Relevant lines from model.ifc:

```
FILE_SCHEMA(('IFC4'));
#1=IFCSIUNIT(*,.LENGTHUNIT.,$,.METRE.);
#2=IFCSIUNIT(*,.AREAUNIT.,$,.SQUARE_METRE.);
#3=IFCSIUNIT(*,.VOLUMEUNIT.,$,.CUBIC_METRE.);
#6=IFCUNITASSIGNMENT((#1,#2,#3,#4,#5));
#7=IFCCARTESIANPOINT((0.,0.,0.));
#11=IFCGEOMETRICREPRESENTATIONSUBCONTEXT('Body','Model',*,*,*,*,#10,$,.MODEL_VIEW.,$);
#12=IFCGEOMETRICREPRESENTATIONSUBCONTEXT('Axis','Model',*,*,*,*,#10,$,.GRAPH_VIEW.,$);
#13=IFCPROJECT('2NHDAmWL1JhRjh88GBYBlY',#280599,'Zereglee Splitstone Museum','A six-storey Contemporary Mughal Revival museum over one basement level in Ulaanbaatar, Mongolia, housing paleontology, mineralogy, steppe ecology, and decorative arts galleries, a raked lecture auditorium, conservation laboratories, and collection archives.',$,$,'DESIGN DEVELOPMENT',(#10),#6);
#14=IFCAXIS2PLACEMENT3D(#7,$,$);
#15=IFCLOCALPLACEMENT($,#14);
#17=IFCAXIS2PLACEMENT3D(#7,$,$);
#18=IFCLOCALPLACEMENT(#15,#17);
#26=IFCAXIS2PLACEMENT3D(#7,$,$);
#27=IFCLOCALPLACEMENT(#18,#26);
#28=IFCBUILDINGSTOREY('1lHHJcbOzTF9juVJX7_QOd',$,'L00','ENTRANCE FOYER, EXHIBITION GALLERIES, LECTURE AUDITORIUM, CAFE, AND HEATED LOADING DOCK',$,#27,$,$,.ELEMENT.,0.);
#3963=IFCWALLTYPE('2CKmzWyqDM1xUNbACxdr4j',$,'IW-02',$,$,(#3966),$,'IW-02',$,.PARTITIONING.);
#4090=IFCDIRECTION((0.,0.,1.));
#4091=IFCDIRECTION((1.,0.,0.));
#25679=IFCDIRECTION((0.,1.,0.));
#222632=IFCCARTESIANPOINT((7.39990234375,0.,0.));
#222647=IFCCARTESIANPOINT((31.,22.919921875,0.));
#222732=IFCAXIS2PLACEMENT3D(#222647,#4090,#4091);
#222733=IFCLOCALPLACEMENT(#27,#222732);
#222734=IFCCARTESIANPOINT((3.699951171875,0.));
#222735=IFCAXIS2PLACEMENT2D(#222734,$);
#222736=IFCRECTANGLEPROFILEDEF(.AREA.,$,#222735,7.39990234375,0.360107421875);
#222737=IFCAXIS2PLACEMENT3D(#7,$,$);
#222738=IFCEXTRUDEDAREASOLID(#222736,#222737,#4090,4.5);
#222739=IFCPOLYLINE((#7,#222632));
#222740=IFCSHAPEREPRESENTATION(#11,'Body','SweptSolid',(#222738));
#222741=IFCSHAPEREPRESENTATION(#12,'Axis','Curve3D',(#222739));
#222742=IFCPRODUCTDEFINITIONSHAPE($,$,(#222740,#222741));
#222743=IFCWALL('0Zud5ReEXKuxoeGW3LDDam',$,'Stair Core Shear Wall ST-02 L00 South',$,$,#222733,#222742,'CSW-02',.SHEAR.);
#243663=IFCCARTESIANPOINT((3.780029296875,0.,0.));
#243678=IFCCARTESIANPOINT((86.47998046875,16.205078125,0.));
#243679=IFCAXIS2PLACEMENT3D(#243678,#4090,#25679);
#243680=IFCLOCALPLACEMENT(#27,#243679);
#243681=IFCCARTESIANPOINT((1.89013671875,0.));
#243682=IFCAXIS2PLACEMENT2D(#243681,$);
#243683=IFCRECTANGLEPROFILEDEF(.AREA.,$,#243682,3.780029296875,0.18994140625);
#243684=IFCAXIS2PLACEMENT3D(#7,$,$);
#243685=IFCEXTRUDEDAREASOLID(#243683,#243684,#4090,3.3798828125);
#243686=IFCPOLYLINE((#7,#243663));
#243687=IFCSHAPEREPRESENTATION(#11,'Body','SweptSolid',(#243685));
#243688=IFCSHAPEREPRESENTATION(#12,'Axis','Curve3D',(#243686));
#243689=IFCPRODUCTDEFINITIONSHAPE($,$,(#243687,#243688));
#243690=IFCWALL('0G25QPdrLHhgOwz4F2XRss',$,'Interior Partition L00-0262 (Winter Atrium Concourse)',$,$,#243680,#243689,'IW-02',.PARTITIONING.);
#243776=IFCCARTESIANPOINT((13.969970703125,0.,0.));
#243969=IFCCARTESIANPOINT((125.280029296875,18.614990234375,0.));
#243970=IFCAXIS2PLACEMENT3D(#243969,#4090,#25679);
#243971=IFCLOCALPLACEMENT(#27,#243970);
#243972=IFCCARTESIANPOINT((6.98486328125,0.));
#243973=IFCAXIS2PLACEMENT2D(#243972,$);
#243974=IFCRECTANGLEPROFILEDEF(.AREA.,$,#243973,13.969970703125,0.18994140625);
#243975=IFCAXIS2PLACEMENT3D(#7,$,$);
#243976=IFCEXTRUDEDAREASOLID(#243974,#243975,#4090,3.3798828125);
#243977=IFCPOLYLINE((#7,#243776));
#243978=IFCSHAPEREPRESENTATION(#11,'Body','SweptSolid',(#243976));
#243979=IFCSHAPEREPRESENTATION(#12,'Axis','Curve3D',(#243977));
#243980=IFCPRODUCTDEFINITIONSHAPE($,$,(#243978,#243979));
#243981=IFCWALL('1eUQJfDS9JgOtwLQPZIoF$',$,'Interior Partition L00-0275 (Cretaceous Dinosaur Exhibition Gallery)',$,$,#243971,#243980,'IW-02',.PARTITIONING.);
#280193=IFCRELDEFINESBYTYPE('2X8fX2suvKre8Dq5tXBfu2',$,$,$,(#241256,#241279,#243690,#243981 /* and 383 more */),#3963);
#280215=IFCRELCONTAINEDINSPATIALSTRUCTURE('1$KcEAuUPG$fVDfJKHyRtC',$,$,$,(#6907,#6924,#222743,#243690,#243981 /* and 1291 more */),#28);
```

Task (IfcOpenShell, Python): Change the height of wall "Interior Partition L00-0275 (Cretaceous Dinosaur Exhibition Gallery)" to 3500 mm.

```python
import ifcopenshell
import ifcopenshell.geom
import ifcopenshell.util.representation
import ifcopenshell.util.shape
import ifcopenshell.util.unit

model = ifcopenshell.open("model.ifc")
unit_scale = ifcopenshell.util.unit.calculate_unit_scale(model)
settings = ifcopenshell.geom.settings()


def volume(element):
    """Net volume in cubic metres, openings subtracted."""
    shape = ifcopenshell.geom.create_shape(settings, element)
    return ifcopenshell.util.shape.get_volume(shape.geometry)


wall = model.by_guid("1eUQJfDS9JgOtwLQPZIoF$")
before = volume(wall)

body = ifcopenshell.util.representation.get_representation(wall, "Model", "Body")
solid = body.Items[0]
old_height = solid.Depth
solid.Depth = 3.5 / unit_scale
after = volume(wall)

print(f"height {old_height:g} -> {solid.Depth:g}, volume {before:.3f} -> {after:.3f} m3")

model.write("model_v2.ifc")
```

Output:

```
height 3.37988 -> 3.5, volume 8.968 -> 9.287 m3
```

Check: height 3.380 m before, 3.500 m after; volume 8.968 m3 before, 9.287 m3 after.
